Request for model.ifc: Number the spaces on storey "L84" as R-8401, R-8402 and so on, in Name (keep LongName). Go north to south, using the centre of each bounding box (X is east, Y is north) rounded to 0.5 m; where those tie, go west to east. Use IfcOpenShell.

First a look at what the model holds.

```python
import ifcopenshell
import ifcopenshell.util.element
import ifcopenshell.util.placement

model = ifcopenshell.open("model.ifc")
print(model.schema)
storey = next(s for s in model.by_type("IfcBuildingStorey") if s.Name == "L84")
spaces = [e for e in ifcopenshell.util.element.get_decomposition(storey) if e.is_a("IfcSpace")]
for e in sorted(spaces, key=lambda e: e.id()):
    origin = ifcopenshell.util.placement.get_local_placement(e.ObjectPlacement)[:3, 3]
    print(e.id(), e.Name, e.LongName, origin.round(2) + 0.0, sep=" | ")
```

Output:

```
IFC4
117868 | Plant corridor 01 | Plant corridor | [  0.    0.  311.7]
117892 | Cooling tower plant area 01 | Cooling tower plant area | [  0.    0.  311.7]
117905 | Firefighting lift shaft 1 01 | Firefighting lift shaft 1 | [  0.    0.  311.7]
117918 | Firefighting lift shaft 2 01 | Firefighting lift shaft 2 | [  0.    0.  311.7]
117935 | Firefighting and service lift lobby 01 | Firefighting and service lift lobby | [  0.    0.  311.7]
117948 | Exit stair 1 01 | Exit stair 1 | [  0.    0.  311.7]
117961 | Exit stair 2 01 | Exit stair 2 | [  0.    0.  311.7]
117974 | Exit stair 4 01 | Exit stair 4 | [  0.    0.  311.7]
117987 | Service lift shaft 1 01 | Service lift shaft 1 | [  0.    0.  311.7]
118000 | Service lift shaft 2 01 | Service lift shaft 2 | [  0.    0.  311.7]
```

```python
import ifcopenshell
import ifcopenshell.geom
import ifcopenshell.util.element
import ifcopenshell.util.shape

model = ifcopenshell.open("model.ifc")
settings = ifcopenshell.geom.settings()
settings.set("use-world-coords", True)


def centre(element):
    shape = ifcopenshell.geom.create_shape(settings, element)
    return ifcopenshell.util.shape.get_bbox_centroid(shape.geometry)


storey = next(s for s in model.by_type("IfcBuildingStorey") if s.Name == "L84")
spaces = [e for e in ifcopenshell.util.element.get_decomposition(storey) if e.is_a("IfcSpace")]

# Insertion points can sit at a corner or the storey origin, so sort by the geometry (in metres).
centres = {e: centre(e) for e in spaces}
spaces.sort(key=lambda e: (-round(centres[e][1] / 0.5), centres[e][0]))

for i, e in enumerate(spaces, start=1):
    number = f"R-84{i:02d}"
    e.Name = number
    print(e.id(), number)

model.write("model_edited.ifc")
```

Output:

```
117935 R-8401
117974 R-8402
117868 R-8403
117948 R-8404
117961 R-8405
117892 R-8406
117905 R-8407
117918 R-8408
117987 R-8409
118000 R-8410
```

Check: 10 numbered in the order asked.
